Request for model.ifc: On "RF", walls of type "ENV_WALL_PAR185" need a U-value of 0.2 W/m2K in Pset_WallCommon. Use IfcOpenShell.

First a look at what the model holds.

```python
import ifcopenshell
import ifcopenshell.util.element

model = ifcopenshell.open("model.ifc")
print(model.schema)
storey = next(s for s in model.by_type("IfcBuildingStorey") if s.Name == "RF")
walls = [e for e in ifcopenshell.util.element.get_decomposition(storey) if e.is_a("IfcWall")]
seen = {}
for e in walls:
    element_type = ifcopenshell.util.element.get_type(e)
    key = (element_type.Name if element_type != e and element_type else None, ifcopenshell.util.element.get_pset(e, "Pset_WallCommon", "ThermalTransmittance"))
    seen[key] = seen.get(key, 0) + 1
for (name, value), count in sorted(seen.items(), key=str):
    print(count, "x", name, "|", value)
```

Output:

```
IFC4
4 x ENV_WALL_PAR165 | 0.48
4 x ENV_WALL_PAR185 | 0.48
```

```python
import ifcopenshell
import ifcopenshell.api.pset
import ifcopenshell.util.element

model = ifcopenshell.open("model.ifc")

storey = next(s for s in model.by_type("IfcBuildingStorey") if s.Name == "RF")
walls = [e for e in ifcopenshell.util.element.get_decomposition(storey) if e.is_a("IfcWall")]

count = 0
for e in walls:
    element_type = ifcopenshell.util.element.get_type(e)
    if element_type in (None, e) or element_type.Name != "ENV_WALL_PAR185":
        continue
    # add_pset returns the element's existing set when there is one.
    pset = ifcopenshell.api.pset.add_pset(model, product=e, name="Pset_WallCommon")
    ifcopenshell.api.pset.edit_pset(model, pset=pset, properties={"ThermalTransmittance": 0.2})
    count += 1

print(count, "walls updated")

model.write("model_updated.ifc")
```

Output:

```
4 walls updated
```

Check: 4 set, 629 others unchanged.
